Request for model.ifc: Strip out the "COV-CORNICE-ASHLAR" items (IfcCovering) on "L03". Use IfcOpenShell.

First a look at what the model holds.

```python
import ifcopenshell
import ifcopenshell.util.element

model = ifcopenshell.open("model.ifc")
print(model.schema)
storey = next(s for s in model.by_type("IfcBuildingStorey") if s.Name == "L03")
coverings = [e for e in ifcopenshell.util.element.get_decomposition(storey) if e.is_a("IfcCovering")]
seen = {}
for e in coverings:
    element_type = ifcopenshell.util.element.get_type(e)
    name = element_type.Name if element_type not in (None, e) else None
    seen[name] = seen.get(name, 0) + 1
for name, count in sorted(seen.items(), key=str):
    print(count, "x", name)
```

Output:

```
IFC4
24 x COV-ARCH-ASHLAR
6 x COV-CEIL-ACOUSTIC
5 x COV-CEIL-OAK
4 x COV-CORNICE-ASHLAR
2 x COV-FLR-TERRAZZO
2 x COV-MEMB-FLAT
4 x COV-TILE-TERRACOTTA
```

```python
import ifcopenshell
import ifcopenshell.api.root
import ifcopenshell.util.element

model = ifcopenshell.open("model.ifc")

storey = next(s for s in model.by_type("IfcBuildingStorey") if s.Name == "L03")
coverings = [e for e in ifcopenshell.util.element.get_decomposition(storey) if e.is_a("IfcCovering")]
targets = [e for e in coverings if (t := ifcopenshell.util.element.get_type(e)) not in (None, e) and t.Name == "COV-CORNICE-ASHLAR"]

for e in targets:
    ifcopenshell.api.root.remove_product(model, product=e)
print(len(targets), "removed")

model.write("model_v2.ifc")
```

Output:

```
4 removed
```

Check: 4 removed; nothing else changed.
